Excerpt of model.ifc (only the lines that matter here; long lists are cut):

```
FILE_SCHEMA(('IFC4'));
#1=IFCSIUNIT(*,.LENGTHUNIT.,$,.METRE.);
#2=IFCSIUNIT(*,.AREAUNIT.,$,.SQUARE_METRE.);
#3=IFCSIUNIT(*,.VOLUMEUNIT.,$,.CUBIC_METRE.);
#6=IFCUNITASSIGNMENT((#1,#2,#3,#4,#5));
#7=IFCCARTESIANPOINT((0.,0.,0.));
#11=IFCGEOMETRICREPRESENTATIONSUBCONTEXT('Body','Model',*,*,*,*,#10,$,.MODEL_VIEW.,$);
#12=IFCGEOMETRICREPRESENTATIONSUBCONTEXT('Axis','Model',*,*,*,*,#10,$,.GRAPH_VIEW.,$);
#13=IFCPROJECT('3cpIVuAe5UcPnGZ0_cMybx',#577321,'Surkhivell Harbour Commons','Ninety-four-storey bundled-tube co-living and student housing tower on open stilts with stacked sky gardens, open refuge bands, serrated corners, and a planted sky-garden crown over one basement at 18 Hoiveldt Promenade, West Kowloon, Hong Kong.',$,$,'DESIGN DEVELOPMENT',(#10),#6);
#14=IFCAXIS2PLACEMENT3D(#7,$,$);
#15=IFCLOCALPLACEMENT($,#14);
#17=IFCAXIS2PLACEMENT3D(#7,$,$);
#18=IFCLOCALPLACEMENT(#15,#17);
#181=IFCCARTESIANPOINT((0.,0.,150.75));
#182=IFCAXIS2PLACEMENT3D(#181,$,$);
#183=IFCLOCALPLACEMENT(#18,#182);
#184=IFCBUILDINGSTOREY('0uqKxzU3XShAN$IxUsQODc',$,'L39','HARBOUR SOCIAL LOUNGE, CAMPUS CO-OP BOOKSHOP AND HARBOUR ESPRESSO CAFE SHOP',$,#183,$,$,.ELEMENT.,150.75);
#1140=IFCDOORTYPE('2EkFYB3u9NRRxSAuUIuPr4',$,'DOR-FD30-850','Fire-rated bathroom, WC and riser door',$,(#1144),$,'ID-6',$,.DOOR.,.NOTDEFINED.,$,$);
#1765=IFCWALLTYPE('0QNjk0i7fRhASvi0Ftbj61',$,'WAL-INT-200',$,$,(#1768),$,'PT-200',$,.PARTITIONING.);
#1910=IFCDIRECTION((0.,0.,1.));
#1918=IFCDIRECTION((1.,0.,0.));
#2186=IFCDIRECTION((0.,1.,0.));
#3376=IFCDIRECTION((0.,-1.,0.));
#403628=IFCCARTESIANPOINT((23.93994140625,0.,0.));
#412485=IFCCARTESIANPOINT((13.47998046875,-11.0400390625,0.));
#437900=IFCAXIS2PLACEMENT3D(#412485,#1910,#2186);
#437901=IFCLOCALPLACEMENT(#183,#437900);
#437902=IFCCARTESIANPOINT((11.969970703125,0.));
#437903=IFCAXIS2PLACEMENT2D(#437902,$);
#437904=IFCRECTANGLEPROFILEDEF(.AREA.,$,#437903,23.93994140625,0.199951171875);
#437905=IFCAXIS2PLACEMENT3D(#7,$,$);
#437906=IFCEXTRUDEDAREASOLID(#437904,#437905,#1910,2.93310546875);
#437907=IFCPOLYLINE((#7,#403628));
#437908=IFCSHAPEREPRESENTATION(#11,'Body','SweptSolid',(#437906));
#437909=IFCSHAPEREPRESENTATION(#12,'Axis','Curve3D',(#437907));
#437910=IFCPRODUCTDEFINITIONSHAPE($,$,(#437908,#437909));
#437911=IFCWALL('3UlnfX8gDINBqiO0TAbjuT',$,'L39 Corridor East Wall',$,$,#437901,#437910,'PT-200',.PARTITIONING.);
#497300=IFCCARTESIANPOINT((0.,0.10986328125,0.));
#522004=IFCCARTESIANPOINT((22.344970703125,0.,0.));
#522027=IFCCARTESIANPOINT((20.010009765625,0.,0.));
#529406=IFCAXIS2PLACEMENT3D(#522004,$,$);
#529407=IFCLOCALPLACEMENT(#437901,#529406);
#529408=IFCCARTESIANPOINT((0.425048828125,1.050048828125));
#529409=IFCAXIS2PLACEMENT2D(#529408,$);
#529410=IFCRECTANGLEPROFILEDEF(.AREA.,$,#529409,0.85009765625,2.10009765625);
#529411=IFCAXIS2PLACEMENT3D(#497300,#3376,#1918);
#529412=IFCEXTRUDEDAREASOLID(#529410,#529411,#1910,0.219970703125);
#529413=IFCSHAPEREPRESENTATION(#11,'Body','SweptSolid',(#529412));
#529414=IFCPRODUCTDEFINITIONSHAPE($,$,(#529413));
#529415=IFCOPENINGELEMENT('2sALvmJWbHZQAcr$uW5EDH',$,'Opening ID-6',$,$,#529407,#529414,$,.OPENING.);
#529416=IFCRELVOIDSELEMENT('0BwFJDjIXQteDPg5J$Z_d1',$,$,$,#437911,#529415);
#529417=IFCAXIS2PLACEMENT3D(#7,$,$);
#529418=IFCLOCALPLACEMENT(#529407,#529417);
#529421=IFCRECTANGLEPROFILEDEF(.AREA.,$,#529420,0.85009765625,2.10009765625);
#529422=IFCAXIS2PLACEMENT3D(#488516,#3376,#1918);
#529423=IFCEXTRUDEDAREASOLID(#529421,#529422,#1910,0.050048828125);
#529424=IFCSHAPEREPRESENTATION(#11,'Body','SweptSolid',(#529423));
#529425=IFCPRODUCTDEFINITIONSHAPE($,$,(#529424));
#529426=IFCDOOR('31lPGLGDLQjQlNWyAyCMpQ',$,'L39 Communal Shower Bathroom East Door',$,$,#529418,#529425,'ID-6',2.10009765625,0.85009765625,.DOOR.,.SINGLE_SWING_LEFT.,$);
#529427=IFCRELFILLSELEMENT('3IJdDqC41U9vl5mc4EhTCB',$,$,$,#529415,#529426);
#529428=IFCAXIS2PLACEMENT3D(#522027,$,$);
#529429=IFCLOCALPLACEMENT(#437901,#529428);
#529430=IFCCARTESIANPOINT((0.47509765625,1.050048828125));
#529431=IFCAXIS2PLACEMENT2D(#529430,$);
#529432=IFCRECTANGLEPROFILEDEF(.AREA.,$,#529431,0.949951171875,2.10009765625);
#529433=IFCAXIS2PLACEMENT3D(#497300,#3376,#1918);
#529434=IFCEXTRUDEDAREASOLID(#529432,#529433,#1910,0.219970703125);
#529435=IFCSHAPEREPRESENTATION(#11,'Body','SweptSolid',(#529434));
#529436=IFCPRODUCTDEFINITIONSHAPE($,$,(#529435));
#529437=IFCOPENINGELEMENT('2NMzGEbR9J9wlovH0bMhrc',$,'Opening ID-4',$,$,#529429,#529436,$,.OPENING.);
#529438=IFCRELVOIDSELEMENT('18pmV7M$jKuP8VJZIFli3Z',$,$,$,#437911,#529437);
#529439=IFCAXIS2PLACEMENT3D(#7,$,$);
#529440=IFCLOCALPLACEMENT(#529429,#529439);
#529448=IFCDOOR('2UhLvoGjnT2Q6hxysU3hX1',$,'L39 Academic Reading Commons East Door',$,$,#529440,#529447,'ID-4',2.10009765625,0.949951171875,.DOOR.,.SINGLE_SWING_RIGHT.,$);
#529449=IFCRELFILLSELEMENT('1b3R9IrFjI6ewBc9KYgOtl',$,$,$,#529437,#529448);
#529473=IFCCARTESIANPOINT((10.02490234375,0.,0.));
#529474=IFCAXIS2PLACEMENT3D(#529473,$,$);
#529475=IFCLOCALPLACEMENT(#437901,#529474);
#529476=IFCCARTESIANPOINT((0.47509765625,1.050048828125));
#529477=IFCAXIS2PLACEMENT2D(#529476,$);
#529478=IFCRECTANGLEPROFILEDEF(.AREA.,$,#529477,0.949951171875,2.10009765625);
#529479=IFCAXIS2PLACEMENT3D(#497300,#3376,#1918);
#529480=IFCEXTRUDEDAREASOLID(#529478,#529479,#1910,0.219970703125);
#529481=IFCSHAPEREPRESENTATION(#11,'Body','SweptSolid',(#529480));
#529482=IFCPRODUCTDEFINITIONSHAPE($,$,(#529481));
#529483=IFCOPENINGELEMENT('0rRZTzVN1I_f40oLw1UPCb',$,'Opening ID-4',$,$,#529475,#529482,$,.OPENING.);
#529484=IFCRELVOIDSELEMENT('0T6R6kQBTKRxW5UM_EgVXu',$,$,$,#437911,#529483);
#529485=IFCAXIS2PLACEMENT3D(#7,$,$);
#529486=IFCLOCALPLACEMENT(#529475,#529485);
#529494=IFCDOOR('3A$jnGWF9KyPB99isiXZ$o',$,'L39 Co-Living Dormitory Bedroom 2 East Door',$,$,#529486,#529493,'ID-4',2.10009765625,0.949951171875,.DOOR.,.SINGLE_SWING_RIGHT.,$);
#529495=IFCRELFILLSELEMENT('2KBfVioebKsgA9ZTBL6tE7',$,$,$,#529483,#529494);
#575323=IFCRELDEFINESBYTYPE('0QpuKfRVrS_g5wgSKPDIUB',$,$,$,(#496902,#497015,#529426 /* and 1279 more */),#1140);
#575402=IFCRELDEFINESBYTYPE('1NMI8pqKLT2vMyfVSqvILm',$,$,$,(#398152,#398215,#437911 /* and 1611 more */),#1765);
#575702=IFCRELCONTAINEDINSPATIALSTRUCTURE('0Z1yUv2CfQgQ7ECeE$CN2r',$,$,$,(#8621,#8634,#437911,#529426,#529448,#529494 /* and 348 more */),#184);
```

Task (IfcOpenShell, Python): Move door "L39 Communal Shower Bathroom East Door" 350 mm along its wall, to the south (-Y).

```python
import ifcopenshell
import ifcopenshell.api.geometry
import ifcopenshell.util.placement
import ifcopenshell.util.unit

model = ifcopenshell.open("model.ifc")
unit_scale = ifcopenshell.util.unit.calculate_unit_scale(model)

door = model.by_guid("31lPGLGDLQjQlNWyAyCMpQ")
opening = door.FillsVoids[0].RelatingOpeningElement
wall = opening.VoidsElements[0].RelatingBuildingElement

wall_matrix = ifcopenshell.util.placement.get_local_placement(wall.ObjectPlacement)
shift = wall_matrix[:3, 0] * -0.35 / unit_scale
before = ifcopenshell.util.placement.get_local_placement(door.ObjectPlacement)[:3, 3].copy()

# The door is placed relative to its opening, so it follows when the opening moves.
matrix = ifcopenshell.util.placement.get_local_placement(opening.ObjectPlacement)
matrix[:3, 3] += shift
ifcopenshell.api.geometry.edit_object_placement(
    model, product=opening, matrix=matrix, is_si=False, should_transform_children=True
)

after = ifcopenshell.util.placement.get_local_placement(door.ObjectPlacement)[:3, 3]
print("door moved by", (after - before).round(3) + 0.0)

model.write("model_updated.ifc")
```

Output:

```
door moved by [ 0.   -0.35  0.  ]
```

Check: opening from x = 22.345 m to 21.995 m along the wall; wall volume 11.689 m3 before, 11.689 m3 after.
